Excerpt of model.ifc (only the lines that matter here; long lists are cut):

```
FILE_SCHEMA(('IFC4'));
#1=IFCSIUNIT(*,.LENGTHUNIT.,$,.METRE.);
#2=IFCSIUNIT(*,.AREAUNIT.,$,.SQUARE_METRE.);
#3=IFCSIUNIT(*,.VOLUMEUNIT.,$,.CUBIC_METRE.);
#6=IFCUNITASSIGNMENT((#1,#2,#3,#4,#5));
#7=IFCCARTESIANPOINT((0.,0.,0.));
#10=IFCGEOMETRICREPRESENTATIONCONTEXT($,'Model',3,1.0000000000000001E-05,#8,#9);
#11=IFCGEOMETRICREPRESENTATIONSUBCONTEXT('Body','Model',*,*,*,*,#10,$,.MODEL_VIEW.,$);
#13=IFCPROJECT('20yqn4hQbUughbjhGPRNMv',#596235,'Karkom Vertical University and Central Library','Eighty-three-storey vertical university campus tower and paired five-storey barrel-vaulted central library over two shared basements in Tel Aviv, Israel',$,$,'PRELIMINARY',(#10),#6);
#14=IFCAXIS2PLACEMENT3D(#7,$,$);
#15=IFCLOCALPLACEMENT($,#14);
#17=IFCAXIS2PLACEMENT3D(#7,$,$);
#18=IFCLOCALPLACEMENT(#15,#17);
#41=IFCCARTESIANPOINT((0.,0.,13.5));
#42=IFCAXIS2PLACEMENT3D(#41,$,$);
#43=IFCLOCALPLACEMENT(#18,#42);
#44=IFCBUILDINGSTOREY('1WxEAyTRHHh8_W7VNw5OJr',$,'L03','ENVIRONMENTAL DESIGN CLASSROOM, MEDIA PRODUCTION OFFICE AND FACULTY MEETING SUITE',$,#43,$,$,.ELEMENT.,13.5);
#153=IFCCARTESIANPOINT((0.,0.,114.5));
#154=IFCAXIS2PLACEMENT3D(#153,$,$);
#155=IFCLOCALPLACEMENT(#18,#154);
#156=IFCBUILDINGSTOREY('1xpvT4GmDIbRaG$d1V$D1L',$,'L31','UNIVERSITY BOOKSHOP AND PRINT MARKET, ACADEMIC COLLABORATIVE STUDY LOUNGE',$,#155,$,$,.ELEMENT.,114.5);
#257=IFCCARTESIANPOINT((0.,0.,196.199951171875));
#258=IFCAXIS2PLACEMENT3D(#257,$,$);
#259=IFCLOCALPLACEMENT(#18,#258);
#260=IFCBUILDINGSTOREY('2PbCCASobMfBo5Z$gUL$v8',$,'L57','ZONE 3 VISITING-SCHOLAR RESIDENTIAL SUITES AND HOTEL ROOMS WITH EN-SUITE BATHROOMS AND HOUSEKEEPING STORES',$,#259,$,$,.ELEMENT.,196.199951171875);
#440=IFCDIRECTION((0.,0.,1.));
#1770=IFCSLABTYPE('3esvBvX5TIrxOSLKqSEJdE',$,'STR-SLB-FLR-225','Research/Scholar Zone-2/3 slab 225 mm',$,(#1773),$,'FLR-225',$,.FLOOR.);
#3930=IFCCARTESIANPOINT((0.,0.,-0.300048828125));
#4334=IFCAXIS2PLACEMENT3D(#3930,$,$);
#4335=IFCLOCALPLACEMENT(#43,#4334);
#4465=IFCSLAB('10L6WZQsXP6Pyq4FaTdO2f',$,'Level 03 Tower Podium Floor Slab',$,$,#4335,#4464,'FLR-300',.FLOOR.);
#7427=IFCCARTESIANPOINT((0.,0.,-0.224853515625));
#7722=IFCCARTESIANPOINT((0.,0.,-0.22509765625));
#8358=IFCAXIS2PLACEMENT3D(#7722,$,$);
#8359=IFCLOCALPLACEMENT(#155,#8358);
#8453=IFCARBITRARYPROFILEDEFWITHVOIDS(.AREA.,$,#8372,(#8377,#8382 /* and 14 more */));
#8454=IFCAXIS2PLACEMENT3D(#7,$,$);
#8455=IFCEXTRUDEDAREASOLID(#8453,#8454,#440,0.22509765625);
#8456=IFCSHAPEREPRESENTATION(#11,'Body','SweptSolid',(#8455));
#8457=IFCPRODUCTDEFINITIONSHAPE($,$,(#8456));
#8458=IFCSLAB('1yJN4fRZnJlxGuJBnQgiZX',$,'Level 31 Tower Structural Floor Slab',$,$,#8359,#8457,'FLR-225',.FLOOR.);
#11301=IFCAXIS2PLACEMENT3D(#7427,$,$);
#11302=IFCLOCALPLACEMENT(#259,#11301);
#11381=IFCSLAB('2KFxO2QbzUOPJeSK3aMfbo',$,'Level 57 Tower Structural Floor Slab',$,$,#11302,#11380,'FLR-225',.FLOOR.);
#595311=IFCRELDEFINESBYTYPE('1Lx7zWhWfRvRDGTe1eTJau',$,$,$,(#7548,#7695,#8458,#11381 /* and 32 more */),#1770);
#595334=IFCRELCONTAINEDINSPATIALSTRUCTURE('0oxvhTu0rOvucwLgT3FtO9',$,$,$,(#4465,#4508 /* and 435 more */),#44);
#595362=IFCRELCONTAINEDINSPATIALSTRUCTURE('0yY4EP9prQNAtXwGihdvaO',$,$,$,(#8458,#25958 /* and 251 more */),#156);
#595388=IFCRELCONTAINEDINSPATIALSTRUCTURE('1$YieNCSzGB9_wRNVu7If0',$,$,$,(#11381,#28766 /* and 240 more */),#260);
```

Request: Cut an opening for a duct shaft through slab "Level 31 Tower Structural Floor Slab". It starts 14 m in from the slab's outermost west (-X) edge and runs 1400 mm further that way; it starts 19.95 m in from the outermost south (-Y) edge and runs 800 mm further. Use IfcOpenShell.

```python
import numpy as np
import ifcopenshell
import ifcopenshell.api.feature
import ifcopenshell.api.geometry
import ifcopenshell.api.root
import ifcopenshell.geom
import ifcopenshell.util.placement
import ifcopenshell.util.representation
import ifcopenshell.util.shape
import ifcopenshell.util.unit

model = ifcopenshell.open("model.ifc")
unit_scale = ifcopenshell.util.unit.calculate_unit_scale(model)
settings = ifcopenshell.geom.settings()


def volume(element):
    """Net volume in cubic metres, openings subtracted."""
    shape = ifcopenshell.geom.create_shape(settings, element)
    return ifcopenshell.util.shape.get_volume(shape.geometry)


slab = model.by_guid("1yJN4fRZnJlxGuJBnQgiZX")
before = volume(slab)

# Extent in the slab's own axes, in metres. The edges named are its -X and -Y sides.
slab_shape = ifcopenshell.geom.create_shape(settings, slab)
vertices = ifcopenshell.util.shape.get_vertices(slab_shape.geometry)
x_min, y_min, bottom = vertices.min(axis=0)
top = vertices[:, 2].max()

opening = ifcopenshell.api.root.create_entity(model, ifc_class="IfcOpeningElement", name="Duct shaft opening", predefined_type="OPENING")
context = ifcopenshell.util.representation.get_context(model, "Model", "Body", "MODEL_VIEW")
width, depth = 1.4, 0.8
outline = [(0.0, 0.0), (width, 0.0), (width, depth), (0.0, depth), (0.0, 0.0)]
# Overshoot both faces by 50 mm so the cut is clean.
shape = ifcopenshell.api.geometry.add_slab_representation(
    model, context=context, depth=top - bottom + 0.1, polyline=outline
)
ifcopenshell.api.geometry.assign_representation(model, product=opening, representation=shape)

matrix = ifcopenshell.util.placement.get_local_placement(slab.ObjectPlacement)
matrix[:, 3] = matrix @ np.append(np.array([x_min + 14, y_min + 19.95, bottom - 0.05]) / unit_scale, 1.0)
ifcopenshell.api.geometry.edit_object_placement(model, product=opening, matrix=matrix, is_si=False)
ifcopenshell.api.feature.add_feature(model, feature=opening, element=slab)

after = volume(slab)

print(f"slab volume {before:.3f} -> {after:.3f} m3")

model.write("model_edited.ifc")
```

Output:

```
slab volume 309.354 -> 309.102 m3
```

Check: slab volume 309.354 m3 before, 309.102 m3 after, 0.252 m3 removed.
